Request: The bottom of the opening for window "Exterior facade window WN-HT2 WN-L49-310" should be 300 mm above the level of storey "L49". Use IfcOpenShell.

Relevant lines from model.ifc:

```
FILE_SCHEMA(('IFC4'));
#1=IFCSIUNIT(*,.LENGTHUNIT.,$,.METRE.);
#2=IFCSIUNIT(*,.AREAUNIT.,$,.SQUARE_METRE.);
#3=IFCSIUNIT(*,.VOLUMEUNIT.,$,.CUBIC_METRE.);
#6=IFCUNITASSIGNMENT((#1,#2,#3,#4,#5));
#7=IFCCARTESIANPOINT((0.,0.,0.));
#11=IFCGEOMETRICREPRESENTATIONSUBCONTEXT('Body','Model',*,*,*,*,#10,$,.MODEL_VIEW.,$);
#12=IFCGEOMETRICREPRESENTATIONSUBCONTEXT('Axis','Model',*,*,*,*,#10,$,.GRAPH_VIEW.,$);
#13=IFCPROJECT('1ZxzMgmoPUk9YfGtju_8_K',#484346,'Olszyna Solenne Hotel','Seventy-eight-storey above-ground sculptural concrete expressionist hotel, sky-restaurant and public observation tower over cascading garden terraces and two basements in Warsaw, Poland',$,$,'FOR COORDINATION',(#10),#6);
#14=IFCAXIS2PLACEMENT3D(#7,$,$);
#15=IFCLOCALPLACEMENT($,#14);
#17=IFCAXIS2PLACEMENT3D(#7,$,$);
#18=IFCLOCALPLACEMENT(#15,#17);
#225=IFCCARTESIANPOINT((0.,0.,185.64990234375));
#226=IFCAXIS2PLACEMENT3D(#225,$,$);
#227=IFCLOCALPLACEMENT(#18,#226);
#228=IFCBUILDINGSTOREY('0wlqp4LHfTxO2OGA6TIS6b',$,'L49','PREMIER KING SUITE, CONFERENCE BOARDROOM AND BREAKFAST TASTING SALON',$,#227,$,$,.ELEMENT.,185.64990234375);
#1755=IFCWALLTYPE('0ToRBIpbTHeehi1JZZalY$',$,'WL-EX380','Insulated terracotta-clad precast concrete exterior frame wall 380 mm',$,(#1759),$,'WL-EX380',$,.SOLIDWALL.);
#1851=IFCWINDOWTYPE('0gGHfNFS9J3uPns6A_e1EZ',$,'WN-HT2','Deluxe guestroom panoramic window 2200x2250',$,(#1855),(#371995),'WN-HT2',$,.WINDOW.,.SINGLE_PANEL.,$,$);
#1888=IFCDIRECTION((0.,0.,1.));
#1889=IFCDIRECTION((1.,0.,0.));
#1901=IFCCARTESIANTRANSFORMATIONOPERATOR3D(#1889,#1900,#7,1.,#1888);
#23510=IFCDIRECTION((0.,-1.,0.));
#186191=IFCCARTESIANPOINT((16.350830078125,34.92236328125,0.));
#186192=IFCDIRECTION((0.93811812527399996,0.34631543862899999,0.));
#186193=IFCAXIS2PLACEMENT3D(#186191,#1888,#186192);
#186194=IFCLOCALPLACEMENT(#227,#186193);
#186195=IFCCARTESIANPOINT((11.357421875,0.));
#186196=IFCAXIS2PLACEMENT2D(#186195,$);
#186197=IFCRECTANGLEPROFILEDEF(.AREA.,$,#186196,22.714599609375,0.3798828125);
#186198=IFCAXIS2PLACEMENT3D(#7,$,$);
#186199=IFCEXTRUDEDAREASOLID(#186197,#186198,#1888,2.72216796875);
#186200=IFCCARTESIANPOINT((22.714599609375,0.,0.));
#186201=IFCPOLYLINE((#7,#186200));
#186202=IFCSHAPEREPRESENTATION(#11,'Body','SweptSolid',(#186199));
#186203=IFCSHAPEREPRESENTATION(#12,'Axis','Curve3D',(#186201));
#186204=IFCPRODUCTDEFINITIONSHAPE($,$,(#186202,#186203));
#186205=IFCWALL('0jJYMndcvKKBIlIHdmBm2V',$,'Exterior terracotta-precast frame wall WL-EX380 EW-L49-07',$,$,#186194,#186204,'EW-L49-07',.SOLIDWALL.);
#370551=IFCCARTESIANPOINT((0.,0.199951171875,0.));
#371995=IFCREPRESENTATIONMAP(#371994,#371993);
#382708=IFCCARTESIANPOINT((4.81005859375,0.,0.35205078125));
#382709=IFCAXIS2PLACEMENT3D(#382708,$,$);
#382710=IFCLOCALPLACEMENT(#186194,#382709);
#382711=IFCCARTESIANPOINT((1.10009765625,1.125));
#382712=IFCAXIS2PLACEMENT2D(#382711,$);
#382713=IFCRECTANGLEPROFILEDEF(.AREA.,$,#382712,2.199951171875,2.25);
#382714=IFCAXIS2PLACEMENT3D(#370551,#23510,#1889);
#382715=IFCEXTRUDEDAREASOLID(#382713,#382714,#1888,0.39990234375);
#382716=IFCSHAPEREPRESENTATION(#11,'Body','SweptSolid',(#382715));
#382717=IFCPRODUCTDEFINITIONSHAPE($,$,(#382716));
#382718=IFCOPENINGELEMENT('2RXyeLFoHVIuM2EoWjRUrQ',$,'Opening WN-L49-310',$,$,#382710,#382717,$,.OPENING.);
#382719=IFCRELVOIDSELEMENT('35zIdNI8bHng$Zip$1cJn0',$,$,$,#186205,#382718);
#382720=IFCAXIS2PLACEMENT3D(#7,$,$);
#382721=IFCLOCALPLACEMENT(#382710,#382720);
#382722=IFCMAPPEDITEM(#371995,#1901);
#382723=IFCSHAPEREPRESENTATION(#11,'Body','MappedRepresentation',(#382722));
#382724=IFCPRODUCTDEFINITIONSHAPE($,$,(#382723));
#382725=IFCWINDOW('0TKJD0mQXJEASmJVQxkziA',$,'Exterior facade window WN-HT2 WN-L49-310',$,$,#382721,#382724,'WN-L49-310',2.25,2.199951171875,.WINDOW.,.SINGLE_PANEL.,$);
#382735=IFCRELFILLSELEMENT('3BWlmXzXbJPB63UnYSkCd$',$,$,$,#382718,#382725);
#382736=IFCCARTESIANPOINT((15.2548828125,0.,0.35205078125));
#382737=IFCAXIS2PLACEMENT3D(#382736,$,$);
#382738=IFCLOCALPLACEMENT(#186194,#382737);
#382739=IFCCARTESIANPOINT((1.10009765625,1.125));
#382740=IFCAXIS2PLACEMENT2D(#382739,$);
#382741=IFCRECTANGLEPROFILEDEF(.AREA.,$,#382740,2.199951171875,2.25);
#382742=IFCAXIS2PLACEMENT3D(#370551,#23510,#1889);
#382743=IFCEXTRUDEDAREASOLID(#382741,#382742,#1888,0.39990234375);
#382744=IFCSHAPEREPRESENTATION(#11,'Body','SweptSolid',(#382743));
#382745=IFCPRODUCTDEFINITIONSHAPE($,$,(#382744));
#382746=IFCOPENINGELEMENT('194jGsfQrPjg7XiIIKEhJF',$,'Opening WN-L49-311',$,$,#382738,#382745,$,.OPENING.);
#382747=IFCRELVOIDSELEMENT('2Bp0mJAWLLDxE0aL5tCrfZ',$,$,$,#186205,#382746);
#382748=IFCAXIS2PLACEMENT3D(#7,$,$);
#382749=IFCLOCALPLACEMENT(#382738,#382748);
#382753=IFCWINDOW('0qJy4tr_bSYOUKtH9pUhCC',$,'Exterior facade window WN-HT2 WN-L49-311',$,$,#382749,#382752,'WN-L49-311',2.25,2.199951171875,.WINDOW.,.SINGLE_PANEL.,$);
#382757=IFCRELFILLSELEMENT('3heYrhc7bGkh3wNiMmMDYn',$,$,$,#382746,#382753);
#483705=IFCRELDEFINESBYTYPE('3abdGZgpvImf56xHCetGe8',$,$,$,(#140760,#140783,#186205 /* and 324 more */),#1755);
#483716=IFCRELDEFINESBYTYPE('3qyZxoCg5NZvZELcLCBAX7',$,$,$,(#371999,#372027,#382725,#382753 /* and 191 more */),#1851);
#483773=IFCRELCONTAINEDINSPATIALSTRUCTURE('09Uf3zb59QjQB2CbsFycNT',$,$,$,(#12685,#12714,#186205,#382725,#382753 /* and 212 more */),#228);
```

```python
import numpy as np
import ifcopenshell
import ifcopenshell.api.geometry
import ifcopenshell.geom
import ifcopenshell.util.element
import ifcopenshell.util.placement
import ifcopenshell.util.shape
import ifcopenshell.util.unit

model = ifcopenshell.open("model.ifc")
unit_scale = ifcopenshell.util.unit.calculate_unit_scale(model)

window = model.by_guid("0TKJD0mQXJEASmJVQxkziA")
opening = window.FillsVoids[0].RelatingOpeningElement
storey = ifcopenshell.util.element.get_container(window, ifc_class="IfcBuildingStorey")
level = ifcopenshell.util.placement.get_local_placement(storey.ObjectPlacement)[2, 3]

# The opening's origin need not be at the sill, so measure its lowest point.
shape = ifcopenshell.geom.create_shape(ifcopenshell.geom.settings(), opening)
bottom = ifcopenshell.util.shape.get_shape_bottom_elevation(shape, shape.geometry) / unit_scale
dz = level + 0.3 - bottom

shift = np.array([0.0, 0.0, dz])
# The window is placed relative to its opening, so it follows when the opening moves.
matrix = ifcopenshell.util.placement.get_local_placement(opening.ObjectPlacement)
matrix[:3, 3] += shift
ifcopenshell.api.geometry.edit_object_placement(
    model, product=opening, matrix=matrix, is_si=False, should_transform_children=True
)

print(f"moved by {dz * unit_scale:+.3f} m")

model.write("model_updated.ifc")
```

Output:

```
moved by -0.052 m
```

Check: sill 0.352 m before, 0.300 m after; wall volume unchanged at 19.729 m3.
